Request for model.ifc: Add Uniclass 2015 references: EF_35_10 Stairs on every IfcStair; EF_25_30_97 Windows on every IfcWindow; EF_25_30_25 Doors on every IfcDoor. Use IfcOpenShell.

First a look at what the model holds.

```python
import ifcopenshell

model = ifcopenshell.open("model.ifc")
print(model.schema)
print("classifications:", [c.Name for c in model.by_type("IfcClassification")])
for ifc_class in ("IfcDoor", "IfcRoof", "IfcStair", "IfcWall", "IfcWindow"):
    print(ifc_class, len(model.by_type(ifc_class)))
```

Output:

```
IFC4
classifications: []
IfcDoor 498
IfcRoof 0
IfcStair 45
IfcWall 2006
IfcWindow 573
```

```python
import ifcopenshell
import ifcopenshell.api.classification

model = ifcopenshell.open("model.ifc")

system = ifcopenshell.api.classification.add_classification(model, classification="Uniclass 2015")

codes = {
    "IfcStair": ("EF_35_10", "Stairs"),
    "IfcWindow": ("EF_25_30_97", "Windows"),
    "IfcDoor": ("EF_25_30_25", "Doors"),
}
for ifc_class, (code, name) in codes.items():
    products = model.by_type(ifc_class)
    ifcopenshell.api.classification.add_reference(
        model, products=products, classification=system, identification=code, name=name
    )
    print(code, len(products))

model.write("model_rev.ifc")
```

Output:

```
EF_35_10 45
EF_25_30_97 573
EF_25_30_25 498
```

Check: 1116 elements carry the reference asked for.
